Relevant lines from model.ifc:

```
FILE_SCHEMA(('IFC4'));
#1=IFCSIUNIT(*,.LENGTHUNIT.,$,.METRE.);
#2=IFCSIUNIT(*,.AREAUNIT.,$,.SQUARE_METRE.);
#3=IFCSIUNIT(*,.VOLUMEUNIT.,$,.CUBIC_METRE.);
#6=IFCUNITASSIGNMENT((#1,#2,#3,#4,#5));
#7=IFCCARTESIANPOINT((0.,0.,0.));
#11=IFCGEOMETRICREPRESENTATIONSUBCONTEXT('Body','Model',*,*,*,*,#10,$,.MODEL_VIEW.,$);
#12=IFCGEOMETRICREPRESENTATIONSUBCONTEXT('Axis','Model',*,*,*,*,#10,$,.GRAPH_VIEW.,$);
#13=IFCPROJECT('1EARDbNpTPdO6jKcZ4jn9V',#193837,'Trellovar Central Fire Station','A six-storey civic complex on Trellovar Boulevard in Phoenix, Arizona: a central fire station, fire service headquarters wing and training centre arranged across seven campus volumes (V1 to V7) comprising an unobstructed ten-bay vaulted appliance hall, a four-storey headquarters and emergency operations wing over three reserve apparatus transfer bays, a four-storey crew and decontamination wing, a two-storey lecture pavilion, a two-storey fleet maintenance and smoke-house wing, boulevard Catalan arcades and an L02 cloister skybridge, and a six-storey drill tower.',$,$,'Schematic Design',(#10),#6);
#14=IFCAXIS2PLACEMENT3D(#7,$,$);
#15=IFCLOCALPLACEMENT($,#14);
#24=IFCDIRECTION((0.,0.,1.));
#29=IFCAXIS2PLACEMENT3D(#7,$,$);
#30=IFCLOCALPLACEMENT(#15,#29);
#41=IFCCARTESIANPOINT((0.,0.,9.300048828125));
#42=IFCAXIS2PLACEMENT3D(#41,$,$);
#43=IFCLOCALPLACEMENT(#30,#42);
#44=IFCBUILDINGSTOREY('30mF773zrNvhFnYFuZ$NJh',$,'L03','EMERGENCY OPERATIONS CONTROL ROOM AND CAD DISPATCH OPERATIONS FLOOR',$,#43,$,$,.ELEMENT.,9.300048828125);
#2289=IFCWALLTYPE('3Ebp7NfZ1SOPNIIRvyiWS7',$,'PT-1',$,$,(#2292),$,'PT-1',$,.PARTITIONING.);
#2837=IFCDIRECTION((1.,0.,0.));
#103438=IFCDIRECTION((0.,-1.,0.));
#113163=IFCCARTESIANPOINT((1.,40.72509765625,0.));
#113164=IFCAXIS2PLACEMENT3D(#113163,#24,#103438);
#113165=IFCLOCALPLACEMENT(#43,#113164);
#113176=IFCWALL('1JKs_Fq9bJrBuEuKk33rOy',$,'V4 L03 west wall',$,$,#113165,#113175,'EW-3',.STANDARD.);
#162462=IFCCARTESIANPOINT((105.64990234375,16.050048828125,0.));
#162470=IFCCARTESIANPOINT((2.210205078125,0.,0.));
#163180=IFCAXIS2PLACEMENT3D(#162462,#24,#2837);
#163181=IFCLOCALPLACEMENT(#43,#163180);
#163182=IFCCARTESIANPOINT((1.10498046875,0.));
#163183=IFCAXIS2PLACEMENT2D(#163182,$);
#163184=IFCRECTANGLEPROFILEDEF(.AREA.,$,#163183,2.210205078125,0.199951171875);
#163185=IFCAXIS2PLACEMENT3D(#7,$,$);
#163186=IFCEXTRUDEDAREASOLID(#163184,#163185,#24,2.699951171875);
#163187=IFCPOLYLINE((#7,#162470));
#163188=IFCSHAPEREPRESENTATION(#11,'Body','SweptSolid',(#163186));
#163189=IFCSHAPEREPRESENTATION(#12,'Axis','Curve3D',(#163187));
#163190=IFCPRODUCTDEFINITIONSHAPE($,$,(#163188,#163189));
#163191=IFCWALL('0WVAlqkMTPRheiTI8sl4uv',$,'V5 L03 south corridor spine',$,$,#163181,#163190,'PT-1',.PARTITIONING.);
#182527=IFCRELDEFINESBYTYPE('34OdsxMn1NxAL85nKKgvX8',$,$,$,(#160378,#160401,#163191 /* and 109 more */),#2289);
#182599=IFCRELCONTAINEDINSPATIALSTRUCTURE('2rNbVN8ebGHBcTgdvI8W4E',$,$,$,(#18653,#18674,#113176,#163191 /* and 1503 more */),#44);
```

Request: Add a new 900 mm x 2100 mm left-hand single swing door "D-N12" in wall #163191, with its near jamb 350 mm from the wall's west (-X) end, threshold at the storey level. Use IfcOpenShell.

```python
import numpy as np
import ifcopenshell
import ifcopenshell.api.feature
import ifcopenshell.api.geometry
import ifcopenshell.api.root
import ifcopenshell.api.spatial
import ifcopenshell.geom
import ifcopenshell.util.element
import ifcopenshell.util.placement
import ifcopenshell.util.representation
import ifcopenshell.util.shape
import ifcopenshell.util.unit

model = ifcopenshell.open("model.ifc")
unit_scale = ifcopenshell.util.unit.calculate_unit_scale(model)
settings = ifcopenshell.geom.settings()


def volume(element):
    """Net volume in cubic metres, openings subtracted."""
    shape = ifcopenshell.geom.create_shape(settings, element)
    return ifcopenshell.util.shape.get_volume(shape.geometry)


wall = model.by_guid("0WVAlqkMTPRheiTI8sl4uv")
storey = ifcopenshell.util.element.get_container(wall, ifc_class="IfcBuildingStorey")
context = ifcopenshell.util.representation.get_context(model, "Model", "Body", "MODEL_VIEW")
before = volume(wall)

width, height, from_end, sill = 0.9, 2.1, 0.35, 0.0  # metres

# The wall runs along its own X axis, and the end named is its -X end.
wall_shape = ifcopenshell.geom.create_shape(settings, wall)
x, y, z = ifcopenshell.util.shape.get_vertices(wall_shape.geometry).T
start = x.min() + from_end
face, thickness = float(y.min()), float(y.max() - y.min())
wall_matrix = ifcopenshell.util.placement.get_local_placement(wall.ObjectPlacement)
level = ifcopenshell.util.placement.get_local_placement(storey.ObjectPlacement)[2, 3]


def in_wall(x, y):
    """Placement at x, y metres in the wall's axes, at sill height."""
    matrix = wall_matrix.copy()
    matrix[:, 3] = wall_matrix @ np.array([x / unit_scale, y / unit_scale, 0.0, 1.0])
    matrix[2, 3] = level + sill / unit_scale
    return matrix


# Opening: a box that overshoots both wall faces by 50 mm.
opening = ifcopenshell.api.root.create_entity(model, ifc_class="IfcOpeningElement", predefined_type="OPENING")
box = ifcopenshell.api.geometry.add_wall_representation(
    model, context=context, length=width, height=height, thickness=thickness + 0.1
)
ifcopenshell.api.geometry.assign_representation(model, product=opening, representation=box)
ifcopenshell.api.geometry.edit_object_placement(model, product=opening, matrix=in_wall(start, face - 0.05), is_si=False)
ifcopenshell.api.feature.add_feature(model, feature=opening, element=wall)

door = ifcopenshell.api.root.create_entity(model, ifc_class="IfcDoor", name="D-N12", predefined_type="DOOR")
door.OverallWidth, door.OverallHeight = width / unit_scale, height / unit_scale
door.OperationType = "SINGLE_SWING_LEFT"
body = ifcopenshell.api.geometry.add_door_representation(
    model,
    context=context,
    overall_width=door.OverallWidth,
    overall_height=door.OverallHeight,
    operation_type="SINGLE_SWING_LEFT",
    lining_properties={"LiningDepth": thickness / unit_scale, "ThresholdDepth": thickness / unit_scale},
)
ifcopenshell.api.geometry.assign_representation(model, product=door, representation=body)
ifcopenshell.api.spatial.assign_container(model, products=[door], relating_structure=storey)
ifcopenshell.api.feature.add_filling(model, opening=opening, element=door)

# The lining spans the wall, so the door starts at the wall face.
ifcopenshell.api.geometry.edit_object_placement(model, product=door, matrix=in_wall(start, face), is_si=False)

after = volume(wall)

print(f"wall volume {before:.3f} -> {after:.3f} m3")

model.write("model_v2.ifc")
```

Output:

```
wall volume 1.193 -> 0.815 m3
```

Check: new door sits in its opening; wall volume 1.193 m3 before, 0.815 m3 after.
